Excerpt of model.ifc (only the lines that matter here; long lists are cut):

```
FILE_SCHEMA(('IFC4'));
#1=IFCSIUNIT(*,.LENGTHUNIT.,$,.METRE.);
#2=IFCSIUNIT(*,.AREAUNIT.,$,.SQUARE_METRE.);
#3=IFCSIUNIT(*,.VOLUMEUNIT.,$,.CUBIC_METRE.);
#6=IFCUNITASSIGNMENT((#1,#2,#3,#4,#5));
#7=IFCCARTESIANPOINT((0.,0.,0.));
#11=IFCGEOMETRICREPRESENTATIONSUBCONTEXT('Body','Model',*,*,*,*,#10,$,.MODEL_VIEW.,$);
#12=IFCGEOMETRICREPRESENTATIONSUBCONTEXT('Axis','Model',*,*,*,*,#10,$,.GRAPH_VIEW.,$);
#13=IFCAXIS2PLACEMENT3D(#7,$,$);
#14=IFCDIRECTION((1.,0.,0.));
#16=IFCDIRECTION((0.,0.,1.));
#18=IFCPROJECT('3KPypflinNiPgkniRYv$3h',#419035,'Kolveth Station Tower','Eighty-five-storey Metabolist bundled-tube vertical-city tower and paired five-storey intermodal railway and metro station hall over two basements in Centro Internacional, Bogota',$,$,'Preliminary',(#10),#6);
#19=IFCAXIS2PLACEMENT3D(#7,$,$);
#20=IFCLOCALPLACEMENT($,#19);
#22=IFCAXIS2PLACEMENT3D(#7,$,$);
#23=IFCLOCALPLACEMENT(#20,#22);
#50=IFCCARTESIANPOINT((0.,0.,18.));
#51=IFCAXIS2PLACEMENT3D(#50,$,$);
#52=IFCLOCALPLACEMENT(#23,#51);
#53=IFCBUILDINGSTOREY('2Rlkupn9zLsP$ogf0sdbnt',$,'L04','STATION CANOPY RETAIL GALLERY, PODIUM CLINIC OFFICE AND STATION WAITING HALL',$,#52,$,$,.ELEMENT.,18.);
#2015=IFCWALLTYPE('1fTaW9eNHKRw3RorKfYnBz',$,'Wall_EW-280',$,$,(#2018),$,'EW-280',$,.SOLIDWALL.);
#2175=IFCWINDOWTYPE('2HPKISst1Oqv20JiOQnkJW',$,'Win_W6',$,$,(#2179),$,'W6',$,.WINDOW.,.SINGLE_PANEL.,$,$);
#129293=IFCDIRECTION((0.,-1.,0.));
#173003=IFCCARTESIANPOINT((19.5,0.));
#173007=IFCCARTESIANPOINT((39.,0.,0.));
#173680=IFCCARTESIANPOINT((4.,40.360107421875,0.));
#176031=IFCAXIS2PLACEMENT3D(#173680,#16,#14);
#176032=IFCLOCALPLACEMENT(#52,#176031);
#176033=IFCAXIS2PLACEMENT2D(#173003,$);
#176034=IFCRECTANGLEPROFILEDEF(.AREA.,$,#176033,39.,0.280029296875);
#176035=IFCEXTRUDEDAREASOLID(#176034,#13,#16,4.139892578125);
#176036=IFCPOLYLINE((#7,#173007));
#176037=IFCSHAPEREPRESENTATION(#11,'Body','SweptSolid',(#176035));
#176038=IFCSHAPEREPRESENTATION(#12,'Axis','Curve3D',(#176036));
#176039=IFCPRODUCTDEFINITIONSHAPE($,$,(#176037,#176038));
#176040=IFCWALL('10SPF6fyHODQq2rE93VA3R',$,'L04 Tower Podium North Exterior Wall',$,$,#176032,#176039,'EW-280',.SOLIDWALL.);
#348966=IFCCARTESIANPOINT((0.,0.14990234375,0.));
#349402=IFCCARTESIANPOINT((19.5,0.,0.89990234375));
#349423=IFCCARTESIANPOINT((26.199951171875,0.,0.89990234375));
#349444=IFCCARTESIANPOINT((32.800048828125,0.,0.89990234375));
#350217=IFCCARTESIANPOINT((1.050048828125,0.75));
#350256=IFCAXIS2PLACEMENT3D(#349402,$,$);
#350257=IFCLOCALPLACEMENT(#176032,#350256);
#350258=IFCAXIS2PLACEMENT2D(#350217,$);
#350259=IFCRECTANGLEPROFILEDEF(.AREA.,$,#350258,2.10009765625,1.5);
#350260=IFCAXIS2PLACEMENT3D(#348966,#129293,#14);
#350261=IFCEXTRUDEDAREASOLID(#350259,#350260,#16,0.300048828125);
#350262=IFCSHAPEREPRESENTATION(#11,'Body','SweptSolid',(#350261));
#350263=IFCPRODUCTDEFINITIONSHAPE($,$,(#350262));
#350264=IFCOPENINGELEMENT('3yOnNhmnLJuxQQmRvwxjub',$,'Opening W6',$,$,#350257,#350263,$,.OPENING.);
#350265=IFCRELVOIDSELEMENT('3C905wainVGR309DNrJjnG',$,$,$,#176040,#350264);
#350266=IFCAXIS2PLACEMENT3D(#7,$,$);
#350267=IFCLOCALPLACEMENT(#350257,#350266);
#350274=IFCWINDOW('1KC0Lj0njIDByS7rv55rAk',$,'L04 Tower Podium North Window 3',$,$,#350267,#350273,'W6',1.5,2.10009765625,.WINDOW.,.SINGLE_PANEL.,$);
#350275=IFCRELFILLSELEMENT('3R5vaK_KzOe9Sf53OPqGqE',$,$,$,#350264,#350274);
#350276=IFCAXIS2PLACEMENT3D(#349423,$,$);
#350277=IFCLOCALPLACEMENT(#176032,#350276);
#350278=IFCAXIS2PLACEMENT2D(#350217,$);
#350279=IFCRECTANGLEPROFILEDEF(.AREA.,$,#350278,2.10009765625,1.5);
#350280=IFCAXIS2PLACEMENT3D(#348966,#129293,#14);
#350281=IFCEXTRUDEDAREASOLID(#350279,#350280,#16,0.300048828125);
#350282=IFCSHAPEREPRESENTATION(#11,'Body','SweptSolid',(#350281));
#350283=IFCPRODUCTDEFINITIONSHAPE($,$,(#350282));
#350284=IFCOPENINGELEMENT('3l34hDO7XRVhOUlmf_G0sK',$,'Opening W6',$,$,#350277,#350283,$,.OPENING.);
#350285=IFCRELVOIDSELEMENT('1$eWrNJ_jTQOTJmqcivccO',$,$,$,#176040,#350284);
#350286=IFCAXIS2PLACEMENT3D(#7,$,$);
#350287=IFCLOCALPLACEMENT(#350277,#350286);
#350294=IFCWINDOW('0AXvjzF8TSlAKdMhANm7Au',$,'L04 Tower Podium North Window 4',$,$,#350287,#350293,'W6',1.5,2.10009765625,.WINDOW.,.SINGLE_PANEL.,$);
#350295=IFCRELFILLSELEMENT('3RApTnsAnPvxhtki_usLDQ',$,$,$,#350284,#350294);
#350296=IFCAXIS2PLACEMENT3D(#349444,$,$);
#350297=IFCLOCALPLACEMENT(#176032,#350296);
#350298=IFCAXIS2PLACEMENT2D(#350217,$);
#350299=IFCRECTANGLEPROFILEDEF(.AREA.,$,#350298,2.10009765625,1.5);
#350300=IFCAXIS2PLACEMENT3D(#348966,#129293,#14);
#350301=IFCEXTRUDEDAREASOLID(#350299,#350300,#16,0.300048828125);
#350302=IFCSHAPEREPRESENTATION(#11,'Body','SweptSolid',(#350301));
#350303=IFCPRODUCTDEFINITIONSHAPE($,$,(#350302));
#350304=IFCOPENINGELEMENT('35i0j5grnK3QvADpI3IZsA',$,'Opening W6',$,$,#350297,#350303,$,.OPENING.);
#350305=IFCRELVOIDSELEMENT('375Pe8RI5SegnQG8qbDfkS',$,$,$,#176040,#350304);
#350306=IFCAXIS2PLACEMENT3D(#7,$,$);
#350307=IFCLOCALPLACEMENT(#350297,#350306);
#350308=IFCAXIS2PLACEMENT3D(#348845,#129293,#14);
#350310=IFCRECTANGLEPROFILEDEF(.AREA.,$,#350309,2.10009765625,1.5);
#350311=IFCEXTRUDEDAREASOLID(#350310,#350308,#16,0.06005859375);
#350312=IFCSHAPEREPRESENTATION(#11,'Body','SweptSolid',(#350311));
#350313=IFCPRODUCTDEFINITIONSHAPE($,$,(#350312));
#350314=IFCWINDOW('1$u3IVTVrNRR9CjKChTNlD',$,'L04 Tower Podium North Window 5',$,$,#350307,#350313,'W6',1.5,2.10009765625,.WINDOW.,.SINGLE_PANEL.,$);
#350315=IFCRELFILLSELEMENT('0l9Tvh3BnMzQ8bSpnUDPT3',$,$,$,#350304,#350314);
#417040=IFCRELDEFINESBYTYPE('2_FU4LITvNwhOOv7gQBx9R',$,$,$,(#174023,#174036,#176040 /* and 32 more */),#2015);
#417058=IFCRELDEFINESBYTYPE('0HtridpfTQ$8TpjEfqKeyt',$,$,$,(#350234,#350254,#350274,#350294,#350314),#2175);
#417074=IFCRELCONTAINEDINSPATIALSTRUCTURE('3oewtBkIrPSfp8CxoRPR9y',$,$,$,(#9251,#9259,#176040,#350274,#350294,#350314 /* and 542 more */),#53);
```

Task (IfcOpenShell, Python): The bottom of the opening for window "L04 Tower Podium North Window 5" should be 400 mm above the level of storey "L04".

```python
import numpy as np
import ifcopenshell
import ifcopenshell.api.geometry
import ifcopenshell.geom
import ifcopenshell.util.element
import ifcopenshell.util.placement
import ifcopenshell.util.shape
import ifcopenshell.util.unit

model = ifcopenshell.open("model.ifc")
unit_scale = ifcopenshell.util.unit.calculate_unit_scale(model)

window = model.by_guid("1$u3IVTVrNRR9CjKChTNlD")
opening = window.FillsVoids[0].RelatingOpeningElement
storey = ifcopenshell.util.element.get_container(window, ifc_class="IfcBuildingStorey")
level = ifcopenshell.util.placement.get_local_placement(storey.ObjectPlacement)[2, 3]

# The opening's origin need not be at the sill, so measure its lowest point.
shape = ifcopenshell.geom.create_shape(ifcopenshell.geom.settings(), opening)
bottom = ifcopenshell.util.shape.get_shape_bottom_elevation(shape, shape.geometry) / unit_scale
dz = level + 0.4 / unit_scale - bottom

shift = np.array([0.0, 0.0, dz])
# The window is placed relative to its opening, so it follows when the opening moves.
matrix = ifcopenshell.util.placement.get_local_placement(opening.ObjectPlacement)
matrix[:3, 3] += shift
ifcopenshell.api.geometry.edit_object_placement(
    model, product=opening, matrix=matrix, is_si=False, should_transform_children=True
)

print(f"moved by {dz * unit_scale:+.3f} m")

model.write("model_updated.ifc")
```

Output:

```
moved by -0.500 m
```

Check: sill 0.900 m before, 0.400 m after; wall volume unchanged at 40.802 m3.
